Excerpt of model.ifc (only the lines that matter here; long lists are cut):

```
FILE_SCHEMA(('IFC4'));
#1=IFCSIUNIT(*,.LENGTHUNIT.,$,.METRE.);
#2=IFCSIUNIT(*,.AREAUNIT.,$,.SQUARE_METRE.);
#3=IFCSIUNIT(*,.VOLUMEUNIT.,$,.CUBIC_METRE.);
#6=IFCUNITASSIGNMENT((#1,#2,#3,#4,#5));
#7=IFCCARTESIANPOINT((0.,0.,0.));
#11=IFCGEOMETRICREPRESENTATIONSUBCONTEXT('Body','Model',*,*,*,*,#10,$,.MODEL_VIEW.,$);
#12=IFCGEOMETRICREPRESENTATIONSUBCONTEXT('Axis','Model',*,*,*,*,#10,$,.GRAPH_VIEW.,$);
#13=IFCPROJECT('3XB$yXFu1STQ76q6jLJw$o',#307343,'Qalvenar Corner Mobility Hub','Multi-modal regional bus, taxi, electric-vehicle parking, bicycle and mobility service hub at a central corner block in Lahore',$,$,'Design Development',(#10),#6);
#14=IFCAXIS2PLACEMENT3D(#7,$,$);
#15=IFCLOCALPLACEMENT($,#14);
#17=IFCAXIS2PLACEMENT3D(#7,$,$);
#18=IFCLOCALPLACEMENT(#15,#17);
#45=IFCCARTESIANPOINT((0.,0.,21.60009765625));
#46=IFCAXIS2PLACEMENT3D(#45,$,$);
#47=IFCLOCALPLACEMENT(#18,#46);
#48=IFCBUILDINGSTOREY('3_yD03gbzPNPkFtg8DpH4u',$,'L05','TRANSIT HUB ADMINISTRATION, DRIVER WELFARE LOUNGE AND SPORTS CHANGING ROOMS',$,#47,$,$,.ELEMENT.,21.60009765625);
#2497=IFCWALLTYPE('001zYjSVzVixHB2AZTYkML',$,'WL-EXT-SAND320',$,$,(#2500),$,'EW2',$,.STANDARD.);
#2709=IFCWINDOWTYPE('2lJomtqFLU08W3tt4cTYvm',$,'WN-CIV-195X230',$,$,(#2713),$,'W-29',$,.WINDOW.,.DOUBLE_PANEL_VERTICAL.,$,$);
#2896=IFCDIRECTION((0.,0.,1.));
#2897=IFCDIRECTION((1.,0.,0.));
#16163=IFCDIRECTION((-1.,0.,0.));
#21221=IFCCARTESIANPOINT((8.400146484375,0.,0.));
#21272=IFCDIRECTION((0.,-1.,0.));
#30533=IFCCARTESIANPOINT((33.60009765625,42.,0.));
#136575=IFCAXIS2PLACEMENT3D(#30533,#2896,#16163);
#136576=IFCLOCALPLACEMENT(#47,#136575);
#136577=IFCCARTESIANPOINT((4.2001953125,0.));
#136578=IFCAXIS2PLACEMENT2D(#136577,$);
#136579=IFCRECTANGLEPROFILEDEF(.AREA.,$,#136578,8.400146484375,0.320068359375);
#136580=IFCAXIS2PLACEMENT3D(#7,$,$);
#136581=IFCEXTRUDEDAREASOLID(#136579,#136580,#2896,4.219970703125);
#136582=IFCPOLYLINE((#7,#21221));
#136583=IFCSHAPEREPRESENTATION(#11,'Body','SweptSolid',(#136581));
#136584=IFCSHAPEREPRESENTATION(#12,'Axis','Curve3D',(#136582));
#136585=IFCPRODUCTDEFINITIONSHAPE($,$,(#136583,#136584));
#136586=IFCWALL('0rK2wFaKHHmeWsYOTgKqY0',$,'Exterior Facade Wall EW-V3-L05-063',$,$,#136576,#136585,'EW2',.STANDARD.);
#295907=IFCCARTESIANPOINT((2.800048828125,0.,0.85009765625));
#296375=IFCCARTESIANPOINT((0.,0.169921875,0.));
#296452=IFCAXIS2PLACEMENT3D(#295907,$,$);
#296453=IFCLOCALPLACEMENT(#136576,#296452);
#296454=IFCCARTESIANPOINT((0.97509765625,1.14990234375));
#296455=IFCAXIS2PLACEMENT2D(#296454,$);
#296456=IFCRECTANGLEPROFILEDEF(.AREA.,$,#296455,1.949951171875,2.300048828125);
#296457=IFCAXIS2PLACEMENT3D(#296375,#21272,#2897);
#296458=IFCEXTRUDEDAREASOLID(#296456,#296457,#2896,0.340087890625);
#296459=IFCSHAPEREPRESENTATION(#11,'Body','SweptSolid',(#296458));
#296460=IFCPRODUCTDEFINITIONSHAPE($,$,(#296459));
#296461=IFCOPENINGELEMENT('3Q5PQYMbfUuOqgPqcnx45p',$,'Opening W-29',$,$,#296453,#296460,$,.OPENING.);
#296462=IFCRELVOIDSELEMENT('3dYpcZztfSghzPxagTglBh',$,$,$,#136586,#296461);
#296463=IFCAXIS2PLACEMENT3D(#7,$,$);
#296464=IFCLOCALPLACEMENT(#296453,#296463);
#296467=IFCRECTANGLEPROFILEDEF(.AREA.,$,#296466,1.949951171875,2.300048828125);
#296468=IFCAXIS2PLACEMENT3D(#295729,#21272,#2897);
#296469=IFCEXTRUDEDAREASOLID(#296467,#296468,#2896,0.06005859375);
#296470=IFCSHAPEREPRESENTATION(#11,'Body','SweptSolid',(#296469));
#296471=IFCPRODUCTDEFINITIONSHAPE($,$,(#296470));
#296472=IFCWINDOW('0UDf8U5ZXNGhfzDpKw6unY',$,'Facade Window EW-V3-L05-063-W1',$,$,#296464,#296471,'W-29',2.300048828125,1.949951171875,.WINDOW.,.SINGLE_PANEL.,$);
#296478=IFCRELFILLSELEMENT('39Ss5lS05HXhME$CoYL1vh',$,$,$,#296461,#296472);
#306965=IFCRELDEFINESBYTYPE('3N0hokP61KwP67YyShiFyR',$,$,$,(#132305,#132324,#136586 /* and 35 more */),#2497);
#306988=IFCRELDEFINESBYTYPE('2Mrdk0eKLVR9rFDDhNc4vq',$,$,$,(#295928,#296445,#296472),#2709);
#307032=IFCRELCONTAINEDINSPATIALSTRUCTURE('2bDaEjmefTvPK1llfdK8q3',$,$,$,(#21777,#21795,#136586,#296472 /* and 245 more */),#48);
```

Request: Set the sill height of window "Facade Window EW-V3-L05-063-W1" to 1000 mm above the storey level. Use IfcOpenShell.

```python
import numpy as np
import ifcopenshell
import ifcopenshell.api.geometry
import ifcopenshell.geom
import ifcopenshell.util.element
import ifcopenshell.util.placement
import ifcopenshell.util.shape
import ifcopenshell.util.unit

model = ifcopenshell.open("model.ifc")
unit_scale = ifcopenshell.util.unit.calculate_unit_scale(model)

window = model.by_guid("0UDf8U5ZXNGhfzDpKw6unY")
opening = window.FillsVoids[0].RelatingOpeningElement
storey = ifcopenshell.util.element.get_container(window, ifc_class="IfcBuildingStorey")
level = ifcopenshell.util.placement.get_local_placement(storey.ObjectPlacement)[2, 3]

# The opening's origin need not be at the sill, so measure its lowest point.
shape = ifcopenshell.geom.create_shape(ifcopenshell.geom.settings(), opening)
bottom = ifcopenshell.util.shape.get_shape_bottom_elevation(shape, shape.geometry) / unit_scale
dz = level + 1 / unit_scale - bottom

shift = np.array([0.0, 0.0, dz])
# The window is placed relative to its opening, so it follows when the opening moves.
matrix = ifcopenshell.util.placement.get_local_placement(opening.ObjectPlacement)
matrix[:3, 3] += shift
ifcopenshell.api.geometry.edit_object_placement(
    model, product=opening, matrix=matrix, is_si=False, should_transform_children=True
)

print(f"moved by {dz * unit_scale:+.3f} m")

model.write("model_updated.ifc")
```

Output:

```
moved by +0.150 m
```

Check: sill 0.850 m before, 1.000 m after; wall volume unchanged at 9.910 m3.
